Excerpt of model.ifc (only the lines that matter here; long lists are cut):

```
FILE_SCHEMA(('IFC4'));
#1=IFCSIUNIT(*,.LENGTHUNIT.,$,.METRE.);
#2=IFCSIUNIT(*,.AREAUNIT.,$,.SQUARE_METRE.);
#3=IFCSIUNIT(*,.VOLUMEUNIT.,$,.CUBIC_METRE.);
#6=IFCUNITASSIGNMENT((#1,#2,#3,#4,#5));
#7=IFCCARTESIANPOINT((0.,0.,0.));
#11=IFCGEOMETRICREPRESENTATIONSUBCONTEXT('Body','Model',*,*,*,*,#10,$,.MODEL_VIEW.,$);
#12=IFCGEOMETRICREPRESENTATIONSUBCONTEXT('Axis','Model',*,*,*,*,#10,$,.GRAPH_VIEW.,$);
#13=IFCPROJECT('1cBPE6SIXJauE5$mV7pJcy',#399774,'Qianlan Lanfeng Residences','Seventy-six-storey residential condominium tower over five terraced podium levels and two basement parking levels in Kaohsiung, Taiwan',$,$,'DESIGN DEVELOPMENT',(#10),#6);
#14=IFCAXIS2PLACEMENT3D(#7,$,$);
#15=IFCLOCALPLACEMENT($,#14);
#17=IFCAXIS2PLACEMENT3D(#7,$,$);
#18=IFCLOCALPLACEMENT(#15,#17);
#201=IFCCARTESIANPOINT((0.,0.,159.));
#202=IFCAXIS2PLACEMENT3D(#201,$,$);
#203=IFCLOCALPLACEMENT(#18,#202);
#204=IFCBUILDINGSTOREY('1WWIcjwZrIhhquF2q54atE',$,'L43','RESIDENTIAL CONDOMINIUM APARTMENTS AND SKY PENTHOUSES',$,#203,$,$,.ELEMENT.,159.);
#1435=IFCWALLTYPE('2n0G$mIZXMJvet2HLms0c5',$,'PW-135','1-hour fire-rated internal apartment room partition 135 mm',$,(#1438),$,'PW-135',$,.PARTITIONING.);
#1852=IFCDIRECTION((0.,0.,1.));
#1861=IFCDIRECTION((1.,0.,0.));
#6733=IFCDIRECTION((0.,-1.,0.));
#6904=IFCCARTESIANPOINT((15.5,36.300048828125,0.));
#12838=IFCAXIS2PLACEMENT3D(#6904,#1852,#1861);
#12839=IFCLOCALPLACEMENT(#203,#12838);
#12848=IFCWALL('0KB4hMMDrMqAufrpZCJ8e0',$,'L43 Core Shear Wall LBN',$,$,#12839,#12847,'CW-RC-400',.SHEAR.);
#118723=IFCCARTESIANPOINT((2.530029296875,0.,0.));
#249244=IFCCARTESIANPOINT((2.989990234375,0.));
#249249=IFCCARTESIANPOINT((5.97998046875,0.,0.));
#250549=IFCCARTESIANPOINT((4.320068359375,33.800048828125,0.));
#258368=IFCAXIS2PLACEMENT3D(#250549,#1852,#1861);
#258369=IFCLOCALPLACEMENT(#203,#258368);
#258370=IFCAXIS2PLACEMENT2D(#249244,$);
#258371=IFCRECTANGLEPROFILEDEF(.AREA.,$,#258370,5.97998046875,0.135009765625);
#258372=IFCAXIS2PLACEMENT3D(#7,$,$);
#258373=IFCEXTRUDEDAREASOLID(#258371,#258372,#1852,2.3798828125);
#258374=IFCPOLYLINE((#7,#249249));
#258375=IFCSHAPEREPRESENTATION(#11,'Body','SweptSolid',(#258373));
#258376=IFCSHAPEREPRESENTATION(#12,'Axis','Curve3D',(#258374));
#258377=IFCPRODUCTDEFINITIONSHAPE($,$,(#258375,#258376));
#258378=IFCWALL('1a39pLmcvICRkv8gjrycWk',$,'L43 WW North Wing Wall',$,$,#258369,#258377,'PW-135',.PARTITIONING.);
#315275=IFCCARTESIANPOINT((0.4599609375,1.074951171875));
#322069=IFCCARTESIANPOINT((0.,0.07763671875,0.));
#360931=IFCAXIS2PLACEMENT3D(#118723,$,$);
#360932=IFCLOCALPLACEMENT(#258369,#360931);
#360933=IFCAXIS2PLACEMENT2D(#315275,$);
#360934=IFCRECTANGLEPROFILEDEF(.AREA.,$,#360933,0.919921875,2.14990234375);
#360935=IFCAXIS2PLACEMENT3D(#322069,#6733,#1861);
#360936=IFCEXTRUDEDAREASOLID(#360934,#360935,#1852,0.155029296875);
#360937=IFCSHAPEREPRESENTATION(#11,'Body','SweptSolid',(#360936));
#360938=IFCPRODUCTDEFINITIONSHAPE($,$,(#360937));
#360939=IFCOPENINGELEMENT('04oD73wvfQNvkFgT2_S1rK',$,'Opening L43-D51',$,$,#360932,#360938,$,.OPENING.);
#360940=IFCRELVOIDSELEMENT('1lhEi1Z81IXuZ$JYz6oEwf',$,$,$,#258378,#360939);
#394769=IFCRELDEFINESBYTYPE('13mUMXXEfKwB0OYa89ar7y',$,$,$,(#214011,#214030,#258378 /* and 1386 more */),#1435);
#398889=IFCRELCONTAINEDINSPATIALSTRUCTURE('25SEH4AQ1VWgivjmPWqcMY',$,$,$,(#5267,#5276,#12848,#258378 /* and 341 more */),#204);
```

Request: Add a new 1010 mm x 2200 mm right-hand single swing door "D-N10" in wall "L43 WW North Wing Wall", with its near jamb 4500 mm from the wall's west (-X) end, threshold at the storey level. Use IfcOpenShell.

```python
import numpy as np
import ifcopenshell
import ifcopenshell.api.feature
import ifcopenshell.api.geometry
import ifcopenshell.api.root
import ifcopenshell.api.spatial
import ifcopenshell.geom
import ifcopenshell.util.element
import ifcopenshell.util.placement
import ifcopenshell.util.representation
import ifcopenshell.util.shape
import ifcopenshell.util.unit

model = ifcopenshell.open("model.ifc")
unit_scale = ifcopenshell.util.unit.calculate_unit_scale(model)
settings = ifcopenshell.geom.settings()


def volume(element):
    """Net volume in cubic metres, openings subtracted."""
    shape = ifcopenshell.geom.create_shape(settings, element)
    return ifcopenshell.util.shape.get_volume(shape.geometry)


wall = model.by_id(258378)
storey = ifcopenshell.util.element.get_container(wall, ifc_class="IfcBuildingStorey")
context = ifcopenshell.util.representation.get_context(model, "Model", "Body", "MODEL_VIEW")
before = volume(wall)

width, height, from_end, sill = 1.01, 2.2, 4.5, 0.0  # metres

# The wall runs along its own X axis, and the end named is its -X end.
wall_shape = ifcopenshell.geom.create_shape(settings, wall)
x, y, z = ifcopenshell.util.shape.get_vertices(wall_shape.geometry).T
start = x.min() + from_end
face, thickness = float(y.min()), float(y.max() - y.min())
wall_matrix = ifcopenshell.util.placement.get_local_placement(wall.ObjectPlacement)
level = ifcopenshell.util.placement.get_local_placement(storey.ObjectPlacement)[2, 3]


def in_wall(x, y):
    """Placement at x, y metres in the wall's axes, at sill height."""
    matrix = wall_matrix.copy()
    matrix[:, 3] = wall_matrix @ np.array([x / unit_scale, y / unit_scale, 0.0, 1.0])
    matrix[2, 3] = level + sill / unit_scale
    return matrix


# Opening: a box that overshoots both wall faces by 50 mm.
opening = ifcopenshell.api.root.create_entity(model, ifc_class="IfcOpeningElement", predefined_type="OPENING")
box = ifcopenshell.api.geometry.add_wall_representation(
    model, context=context, length=width, height=height, thickness=thickness + 0.1
)
ifcopenshell.api.geometry.assign_representation(model, product=opening, representation=box)
ifcopenshell.api.geometry.edit_object_placement(model, product=opening, matrix=in_wall(start, face - 0.05), is_si=False)
ifcopenshell.api.feature.add_feature(model, feature=opening, element=wall)

door = ifcopenshell.api.root.create_entity(model, ifc_class="IfcDoor", name="D-N10", predefined_type="DOOR")
door.OverallWidth, door.OverallHeight = width / unit_scale, height / unit_scale
door.OperationType = "SINGLE_SWING_RIGHT"
body = ifcopenshell.api.geometry.add_door_representation(
    model,
    context=context,
    overall_width=door.OverallWidth,
    overall_height=door.OverallHeight,
    operation_type="SINGLE_SWING_RIGHT",
    lining_properties={"LiningDepth": thickness / unit_scale, "ThresholdDepth": thickness / unit_scale},
)
ifcopenshell.api.geometry.assign_representation(model, product=door, representation=body)
ifcopenshell.api.spatial.assign_container(model, products=[door], relating_structure=storey)
ifcopenshell.api.feature.add_filling(model, opening=opening, element=door)

# The lining spans the wall, so the door starts at the wall face.
ifcopenshell.api.geometry.edit_object_placement(model, product=door, matrix=in_wall(start, face), is_si=False)

after = volume(wall)

print(f"wall volume {before:.3f} -> {after:.3f} m3")

model.write("model_v2.ifc")
```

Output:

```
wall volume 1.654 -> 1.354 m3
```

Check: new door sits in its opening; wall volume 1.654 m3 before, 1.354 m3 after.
